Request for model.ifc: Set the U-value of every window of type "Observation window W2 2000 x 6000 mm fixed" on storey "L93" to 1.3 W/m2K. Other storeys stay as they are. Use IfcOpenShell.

First a look at what the model holds.

```python
import ifcopenshell
import ifcopenshell.util.element

model = ifcopenshell.open("model.ifc")
print(model.schema)
storey = next(s for s in model.by_type("IfcBuildingStorey") if s.Name == "L93")
windows = [e for e in ifcopenshell.util.element.get_decomposition(storey) if e.is_a("IfcWindow")]
seen = {}
for e in windows:
    element_type = ifcopenshell.util.element.get_type(e)
    key = (element_type.Name if element_type != e and element_type else None, ifcopenshell.util.element.get_pset(e, "Pset_WindowCommon", "ThermalTransmittance"))
    seen[key] = seen.get(key, 0) + 1
for (name, value), count in sorted(seen.items(), key=str):
    print(count, "x", name, "|", value)
```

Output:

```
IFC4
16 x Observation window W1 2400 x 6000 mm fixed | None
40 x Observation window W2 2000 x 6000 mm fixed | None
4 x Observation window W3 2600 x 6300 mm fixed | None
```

```python
import ifcopenshell
import ifcopenshell.api.pset
import ifcopenshell.util.element

model = ifcopenshell.open("model.ifc")

storey = next(s for s in model.by_type("IfcBuildingStorey") if s.Name == "L93")
windows = [e for e in ifcopenshell.util.element.get_decomposition(storey) if e.is_a("IfcWindow")]

count = 0
for e in windows:
    element_type = ifcopenshell.util.element.get_type(e)
    if element_type in (None, e) or element_type.Name != "Observation window W2 2000 x 6000 mm fixed":
        continue
    found = ifcopenshell.util.element.get_pset(e, "Pset_WindowCommon", should_inherit=False)
    if found:
        pset = model.by_id(found["id"])
        if len(ifcopenshell.util.element.get_elements_by_pset(pset)) > 1:
            pset = ifcopenshell.api.pset.unshare_pset(model, products=[e], pset=pset)[0]
    else:
        pset = ifcopenshell.api.pset.add_pset(model, product=e, name="Pset_WindowCommon")
    ifcopenshell.api.pset.edit_pset(model, pset=pset, properties={"ThermalTransmittance": 1.3})
    count += 1

print(count, "windows updated")

model.write("model_edited.ifc")
```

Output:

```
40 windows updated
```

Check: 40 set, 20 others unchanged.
